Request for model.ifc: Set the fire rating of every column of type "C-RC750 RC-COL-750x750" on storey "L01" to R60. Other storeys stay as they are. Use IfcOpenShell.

First a look at what the model holds.

```python
import ifcopenshell
import ifcopenshell.util.element

model = ifcopenshell.open("model.ifc")
print(model.schema)
storey = next(s for s in model.by_type("IfcBuildingStorey") if s.Name == "L01")
columns = [e for e in ifcopenshell.util.element.get_decomposition(storey) if e.is_a("IfcColumn")]
seen = {}
for e in columns:
    element_type = ifcopenshell.util.element.get_type(e)
    key = (element_type.Name if element_type != e and element_type else None, ifcopenshell.util.element.get_pset(e, "Pset_ColumnCommon", "FireRating"))
    seen[key] = seen.get(key, 0) + 1
for (name, value), count in sorted(seen.items(), key=str):
    print(count, "x", name, "|", value)
```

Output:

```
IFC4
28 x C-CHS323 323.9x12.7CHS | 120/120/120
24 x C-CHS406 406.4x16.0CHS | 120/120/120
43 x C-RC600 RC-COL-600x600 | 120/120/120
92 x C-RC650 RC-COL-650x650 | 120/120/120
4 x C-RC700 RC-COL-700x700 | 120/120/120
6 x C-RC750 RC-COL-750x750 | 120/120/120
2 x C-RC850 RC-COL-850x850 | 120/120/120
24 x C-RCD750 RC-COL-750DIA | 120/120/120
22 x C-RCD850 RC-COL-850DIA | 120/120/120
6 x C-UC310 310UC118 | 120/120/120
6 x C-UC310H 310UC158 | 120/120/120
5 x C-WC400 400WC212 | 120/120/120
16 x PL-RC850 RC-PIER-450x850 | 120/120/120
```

```python
import ifcopenshell
import ifcopenshell.api.pset
import ifcopenshell.util.element

model = ifcopenshell.open("model.ifc")

storey = next(s for s in model.by_type("IfcBuildingStorey") if s.Name == "L01")
columns = [e for e in ifcopenshell.util.element.get_decomposition(storey) if e.is_a("IfcColumn")]

count = 0
for e in columns:
    element_type = ifcopenshell.util.element.get_type(e)
    if element_type in (None, e) or element_type.Name != "C-RC750 RC-COL-750x750":
        continue
    # add_pset returns the element's existing set when there is one.
    pset = ifcopenshell.api.pset.add_pset(model, product=e, name="Pset_ColumnCommon")
    ifcopenshell.api.pset.edit_pset(model, pset=pset, properties={"FireRating": "R60"})
    count += 1

print(count, "columns updated")

model.write("model-out.ifc")
```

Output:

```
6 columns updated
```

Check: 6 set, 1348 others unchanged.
